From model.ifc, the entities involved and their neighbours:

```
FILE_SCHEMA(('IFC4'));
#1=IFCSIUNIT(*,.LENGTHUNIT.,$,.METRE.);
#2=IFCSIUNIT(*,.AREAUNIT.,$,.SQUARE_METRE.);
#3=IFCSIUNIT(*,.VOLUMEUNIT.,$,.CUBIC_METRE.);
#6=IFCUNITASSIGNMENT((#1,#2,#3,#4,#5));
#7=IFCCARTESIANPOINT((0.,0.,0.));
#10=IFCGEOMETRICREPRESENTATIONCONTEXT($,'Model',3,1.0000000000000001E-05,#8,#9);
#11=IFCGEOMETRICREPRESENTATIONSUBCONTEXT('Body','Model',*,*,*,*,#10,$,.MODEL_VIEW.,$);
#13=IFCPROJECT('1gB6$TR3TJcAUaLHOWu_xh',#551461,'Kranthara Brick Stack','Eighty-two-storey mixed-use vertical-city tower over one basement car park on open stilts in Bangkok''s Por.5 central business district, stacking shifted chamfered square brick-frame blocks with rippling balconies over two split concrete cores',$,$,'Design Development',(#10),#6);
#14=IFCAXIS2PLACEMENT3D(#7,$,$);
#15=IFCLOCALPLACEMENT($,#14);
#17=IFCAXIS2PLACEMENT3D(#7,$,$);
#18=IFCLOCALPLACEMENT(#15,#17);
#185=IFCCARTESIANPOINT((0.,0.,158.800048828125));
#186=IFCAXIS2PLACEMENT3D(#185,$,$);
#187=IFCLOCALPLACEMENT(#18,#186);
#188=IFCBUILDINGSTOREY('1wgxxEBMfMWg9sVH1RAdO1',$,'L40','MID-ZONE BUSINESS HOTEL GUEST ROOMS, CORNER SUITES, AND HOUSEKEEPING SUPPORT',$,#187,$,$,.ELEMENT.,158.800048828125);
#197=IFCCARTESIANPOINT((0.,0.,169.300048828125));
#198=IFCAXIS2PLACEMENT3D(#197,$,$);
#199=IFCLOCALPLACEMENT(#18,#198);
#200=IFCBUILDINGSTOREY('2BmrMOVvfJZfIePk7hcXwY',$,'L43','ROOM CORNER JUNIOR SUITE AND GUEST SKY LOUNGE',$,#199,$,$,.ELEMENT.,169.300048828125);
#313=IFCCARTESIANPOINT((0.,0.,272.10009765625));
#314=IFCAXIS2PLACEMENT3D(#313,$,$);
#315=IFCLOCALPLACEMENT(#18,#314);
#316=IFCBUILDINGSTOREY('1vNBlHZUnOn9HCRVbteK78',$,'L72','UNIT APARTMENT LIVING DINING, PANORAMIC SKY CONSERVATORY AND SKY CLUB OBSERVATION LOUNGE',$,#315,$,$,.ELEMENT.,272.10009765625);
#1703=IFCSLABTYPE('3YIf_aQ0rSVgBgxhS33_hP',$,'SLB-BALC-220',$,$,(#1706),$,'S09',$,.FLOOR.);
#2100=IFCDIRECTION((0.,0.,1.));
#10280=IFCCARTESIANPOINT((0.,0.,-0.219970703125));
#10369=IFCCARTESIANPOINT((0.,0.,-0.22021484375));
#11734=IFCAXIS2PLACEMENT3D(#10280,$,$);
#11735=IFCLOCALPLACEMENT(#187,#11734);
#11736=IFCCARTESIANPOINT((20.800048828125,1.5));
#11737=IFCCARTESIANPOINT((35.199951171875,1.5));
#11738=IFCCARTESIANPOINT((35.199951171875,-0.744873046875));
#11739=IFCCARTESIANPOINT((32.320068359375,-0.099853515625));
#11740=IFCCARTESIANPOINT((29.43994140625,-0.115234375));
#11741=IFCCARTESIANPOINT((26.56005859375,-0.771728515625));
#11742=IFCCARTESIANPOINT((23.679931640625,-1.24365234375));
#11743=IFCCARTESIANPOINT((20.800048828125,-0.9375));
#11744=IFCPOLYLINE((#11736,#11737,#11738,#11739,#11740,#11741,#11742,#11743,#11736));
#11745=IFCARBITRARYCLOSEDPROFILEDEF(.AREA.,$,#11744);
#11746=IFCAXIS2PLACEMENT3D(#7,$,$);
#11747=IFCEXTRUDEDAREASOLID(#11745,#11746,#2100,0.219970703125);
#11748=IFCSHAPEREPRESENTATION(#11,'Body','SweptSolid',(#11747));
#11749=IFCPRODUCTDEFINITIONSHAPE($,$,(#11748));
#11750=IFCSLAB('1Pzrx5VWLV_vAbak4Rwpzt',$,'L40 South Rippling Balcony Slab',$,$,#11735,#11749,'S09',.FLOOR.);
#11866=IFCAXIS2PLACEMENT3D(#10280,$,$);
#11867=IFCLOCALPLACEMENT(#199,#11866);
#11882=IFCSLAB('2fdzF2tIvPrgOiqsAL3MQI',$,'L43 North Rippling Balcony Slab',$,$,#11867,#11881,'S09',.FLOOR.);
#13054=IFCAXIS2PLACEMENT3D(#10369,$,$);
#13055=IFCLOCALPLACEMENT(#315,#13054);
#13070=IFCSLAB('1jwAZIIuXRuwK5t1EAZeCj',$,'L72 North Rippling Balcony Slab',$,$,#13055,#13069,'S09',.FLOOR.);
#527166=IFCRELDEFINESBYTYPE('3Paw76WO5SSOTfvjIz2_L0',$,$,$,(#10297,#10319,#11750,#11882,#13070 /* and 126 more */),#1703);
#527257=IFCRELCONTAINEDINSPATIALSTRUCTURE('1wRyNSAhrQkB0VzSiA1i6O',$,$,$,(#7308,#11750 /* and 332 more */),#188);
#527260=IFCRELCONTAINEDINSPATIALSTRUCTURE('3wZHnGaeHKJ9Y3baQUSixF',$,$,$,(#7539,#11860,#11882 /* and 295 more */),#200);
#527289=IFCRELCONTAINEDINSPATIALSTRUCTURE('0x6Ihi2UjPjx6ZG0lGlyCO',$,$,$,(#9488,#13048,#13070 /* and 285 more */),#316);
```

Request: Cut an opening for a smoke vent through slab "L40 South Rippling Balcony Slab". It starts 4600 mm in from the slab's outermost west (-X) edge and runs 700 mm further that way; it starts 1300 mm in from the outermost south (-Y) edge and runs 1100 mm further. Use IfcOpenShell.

```python
import numpy as np
import ifcopenshell
import ifcopenshell.api.feature
import ifcopenshell.api.geometry
import ifcopenshell.api.root
import ifcopenshell.geom
import ifcopenshell.util.placement
import ifcopenshell.util.representation
import ifcopenshell.util.shape
import ifcopenshell.util.unit

model = ifcopenshell.open("model.ifc")
unit_scale = ifcopenshell.util.unit.calculate_unit_scale(model)
settings = ifcopenshell.geom.settings()


def volume(element):
    """Net volume in cubic metres, openings subtracted."""
    shape = ifcopenshell.geom.create_shape(settings, element)
    return ifcopenshell.util.shape.get_volume(shape.geometry)


slab = model.by_id(11750)
before = volume(slab)

# Extent in the slab's own axes, in metres. The edges named are its -X and -Y sides.
slab_shape = ifcopenshell.geom.create_shape(settings, slab)
vertices = ifcopenshell.util.shape.get_vertices(slab_shape.geometry)
x_min, y_min, bottom = vertices.min(axis=0)
top = vertices[:, 2].max()

opening = ifcopenshell.api.root.create_entity(model, ifc_class="IfcOpeningElement", name="Smoke vent opening", predefined_type="OPENING")
context = ifcopenshell.util.representation.get_context(model, "Model", "Body", "MODEL_VIEW")
width, depth = 0.7, 1.1
outline = [(0.0, 0.0), (width, 0.0), (width, depth), (0.0, depth), (0.0, 0.0)]
# Overshoot both faces by 50 mm so the cut is clean.
shape = ifcopenshell.api.geometry.add_slab_representation(
    model, context=context, depth=top - bottom + 0.1, polyline=outline
)
ifcopenshell.api.geometry.assign_representation(model, product=opening, representation=shape)

matrix = ifcopenshell.util.placement.get_local_placement(slab.ObjectPlacement)
matrix[:, 3] = matrix @ np.append(np.array([x_min + 4.6, y_min + 1.3, bottom - 0.05]) / unit_scale, 1.0)
ifcopenshell.api.geometry.edit_object_placement(model, product=opening, matrix=matrix, is_si=False)
ifcopenshell.api.feature.add_feature(model, feature=opening, element=slab)

after = volume(slab)

print(f"slab volume {before:.3f} -> {after:.3f} m3")

model.write("model_v2.ifc")
```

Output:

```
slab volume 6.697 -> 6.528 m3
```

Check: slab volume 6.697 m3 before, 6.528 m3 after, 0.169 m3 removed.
